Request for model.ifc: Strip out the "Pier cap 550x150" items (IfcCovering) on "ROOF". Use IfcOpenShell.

First a look at what the model holds.

```python
import ifcopenshell
import ifcopenshell.util.element

model = ifcopenshell.open("model.ifc")
print(model.schema)
storey = next(s for s in model.by_type("IfcBuildingStorey") if s.Name == "ROOF")
coverings = [e for e in ifcopenshell.util.element.get_decomposition(storey) if e.is_a("IfcCovering")]
seen = {}
for e in coverings:
    element_type = ifcopenshell.util.element.get_type(e)
    name = element_type.Name if element_type not in (None, e) else None
    seen[name] = seen.get(name, 0) + 1
for name, count in sorted(seen.items(), key=str):
    print(count, "x", name)
```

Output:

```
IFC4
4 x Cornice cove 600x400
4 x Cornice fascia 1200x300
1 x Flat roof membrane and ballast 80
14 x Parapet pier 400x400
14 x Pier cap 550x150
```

```python
import ifcopenshell
import ifcopenshell.api.root
import ifcopenshell.util.element

model = ifcopenshell.open("model.ifc")

storey = next(s for s in model.by_type("IfcBuildingStorey") if s.Name == "ROOF")
coverings = [e for e in ifcopenshell.util.element.get_decomposition(storey) if e.is_a("IfcCovering")]
targets = [e for e in coverings if (t := ifcopenshell.util.element.get_type(e)) not in (None, e) and t.Name == "Pier cap 550x150"]

for e in targets:
    ifcopenshell.api.root.remove_product(model, product=e)
print(len(targets), "removed")

model.write("model_v2.ifc")
```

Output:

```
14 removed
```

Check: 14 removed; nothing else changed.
